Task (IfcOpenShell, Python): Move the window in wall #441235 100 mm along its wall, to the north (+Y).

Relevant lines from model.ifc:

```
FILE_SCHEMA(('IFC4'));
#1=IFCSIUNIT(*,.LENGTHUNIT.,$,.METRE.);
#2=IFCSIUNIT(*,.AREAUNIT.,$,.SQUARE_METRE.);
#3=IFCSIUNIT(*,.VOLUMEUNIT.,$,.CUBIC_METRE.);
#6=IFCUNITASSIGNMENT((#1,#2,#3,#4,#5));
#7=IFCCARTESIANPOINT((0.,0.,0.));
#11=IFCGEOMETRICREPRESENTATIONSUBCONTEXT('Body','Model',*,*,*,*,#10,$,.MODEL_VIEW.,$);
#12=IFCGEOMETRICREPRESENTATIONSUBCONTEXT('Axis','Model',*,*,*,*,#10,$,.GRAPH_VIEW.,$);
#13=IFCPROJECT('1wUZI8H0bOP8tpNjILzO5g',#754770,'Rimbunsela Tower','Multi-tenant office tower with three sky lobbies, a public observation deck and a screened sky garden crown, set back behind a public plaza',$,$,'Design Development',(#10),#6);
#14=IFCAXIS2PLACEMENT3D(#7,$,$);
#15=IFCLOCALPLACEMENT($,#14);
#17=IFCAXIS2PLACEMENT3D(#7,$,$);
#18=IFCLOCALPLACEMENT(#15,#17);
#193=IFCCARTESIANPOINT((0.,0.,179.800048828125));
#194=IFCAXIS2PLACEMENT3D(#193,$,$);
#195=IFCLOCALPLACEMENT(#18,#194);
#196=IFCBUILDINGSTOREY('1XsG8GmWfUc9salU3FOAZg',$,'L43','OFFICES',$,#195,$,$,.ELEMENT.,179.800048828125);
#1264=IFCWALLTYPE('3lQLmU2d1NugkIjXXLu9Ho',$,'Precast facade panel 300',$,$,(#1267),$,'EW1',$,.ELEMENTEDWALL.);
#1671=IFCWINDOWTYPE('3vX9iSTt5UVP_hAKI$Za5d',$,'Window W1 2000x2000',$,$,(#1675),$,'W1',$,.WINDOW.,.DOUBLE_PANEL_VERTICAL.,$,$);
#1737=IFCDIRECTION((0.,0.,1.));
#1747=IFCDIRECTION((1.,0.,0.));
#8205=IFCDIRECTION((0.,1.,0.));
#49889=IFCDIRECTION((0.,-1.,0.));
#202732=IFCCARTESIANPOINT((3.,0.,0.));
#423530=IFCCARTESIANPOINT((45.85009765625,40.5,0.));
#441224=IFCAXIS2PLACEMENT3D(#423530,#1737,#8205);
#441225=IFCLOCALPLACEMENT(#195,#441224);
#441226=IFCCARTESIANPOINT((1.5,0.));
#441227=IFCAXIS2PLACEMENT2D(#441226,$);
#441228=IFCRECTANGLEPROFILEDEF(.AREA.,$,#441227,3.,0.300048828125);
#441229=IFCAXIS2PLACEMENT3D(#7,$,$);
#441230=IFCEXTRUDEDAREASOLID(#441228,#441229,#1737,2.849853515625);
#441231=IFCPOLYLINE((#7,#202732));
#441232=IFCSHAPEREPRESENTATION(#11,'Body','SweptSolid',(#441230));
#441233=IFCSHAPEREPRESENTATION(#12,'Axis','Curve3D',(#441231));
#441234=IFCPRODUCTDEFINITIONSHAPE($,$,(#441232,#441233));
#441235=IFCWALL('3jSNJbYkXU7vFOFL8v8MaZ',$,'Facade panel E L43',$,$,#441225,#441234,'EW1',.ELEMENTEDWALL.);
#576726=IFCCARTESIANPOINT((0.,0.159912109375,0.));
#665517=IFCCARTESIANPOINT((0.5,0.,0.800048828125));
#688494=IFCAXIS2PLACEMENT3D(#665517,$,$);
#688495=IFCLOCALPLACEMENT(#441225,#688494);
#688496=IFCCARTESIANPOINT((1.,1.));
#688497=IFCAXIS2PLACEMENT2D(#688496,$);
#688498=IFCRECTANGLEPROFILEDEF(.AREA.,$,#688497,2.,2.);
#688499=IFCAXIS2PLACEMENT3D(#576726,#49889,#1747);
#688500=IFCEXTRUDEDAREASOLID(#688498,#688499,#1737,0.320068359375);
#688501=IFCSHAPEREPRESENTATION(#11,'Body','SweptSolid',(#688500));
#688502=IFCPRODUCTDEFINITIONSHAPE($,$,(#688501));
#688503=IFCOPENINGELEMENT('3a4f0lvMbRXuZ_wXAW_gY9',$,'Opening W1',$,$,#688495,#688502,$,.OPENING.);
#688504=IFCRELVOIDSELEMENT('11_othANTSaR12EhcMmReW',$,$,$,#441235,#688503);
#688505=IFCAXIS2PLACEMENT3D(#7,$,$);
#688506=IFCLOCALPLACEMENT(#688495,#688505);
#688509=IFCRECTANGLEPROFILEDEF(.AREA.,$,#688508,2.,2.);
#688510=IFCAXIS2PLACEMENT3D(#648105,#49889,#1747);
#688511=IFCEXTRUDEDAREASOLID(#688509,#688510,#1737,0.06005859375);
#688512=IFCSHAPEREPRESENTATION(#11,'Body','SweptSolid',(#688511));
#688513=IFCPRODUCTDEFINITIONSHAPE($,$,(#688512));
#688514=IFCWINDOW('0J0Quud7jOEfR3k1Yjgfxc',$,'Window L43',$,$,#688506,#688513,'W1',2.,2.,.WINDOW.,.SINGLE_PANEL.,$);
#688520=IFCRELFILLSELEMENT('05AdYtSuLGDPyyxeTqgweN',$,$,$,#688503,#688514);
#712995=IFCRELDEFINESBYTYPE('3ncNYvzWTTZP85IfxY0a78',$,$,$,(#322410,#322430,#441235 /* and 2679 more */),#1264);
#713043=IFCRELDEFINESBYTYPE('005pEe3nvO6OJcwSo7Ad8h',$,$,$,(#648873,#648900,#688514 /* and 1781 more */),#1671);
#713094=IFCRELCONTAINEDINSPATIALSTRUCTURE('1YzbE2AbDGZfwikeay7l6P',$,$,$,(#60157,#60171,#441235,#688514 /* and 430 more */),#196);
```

```python
import ifcopenshell
import ifcopenshell.api.geometry
import ifcopenshell.util.placement
import ifcopenshell.util.unit

model = ifcopenshell.open("model.ifc")
unit_scale = ifcopenshell.util.unit.calculate_unit_scale(model)

window = model.by_guid("0J0Quud7jOEfR3k1Yjgfxc")
opening = window.FillsVoids[0].RelatingOpeningElement
wall = opening.VoidsElements[0].RelatingBuildingElement

wall_matrix = ifcopenshell.util.placement.get_local_placement(wall.ObjectPlacement)
shift = wall_matrix[:3, 0] * 0.1 / unit_scale
before = ifcopenshell.util.placement.get_local_placement(window.ObjectPlacement)[:3, 3].copy()

# The window is placed relative to its opening, so it follows when the opening moves.
matrix = ifcopenshell.util.placement.get_local_placement(opening.ObjectPlacement)
matrix[:3, 3] += shift
ifcopenshell.api.geometry.edit_object_placement(
    model, product=opening, matrix=matrix, is_si=False, should_transform_children=True
)

after = ifcopenshell.util.placement.get_local_placement(window.ObjectPlacement)[:3, 3]
print("window moved by", (after - before).round(3) + 0.0)

model.write("model_v2.ifc")
```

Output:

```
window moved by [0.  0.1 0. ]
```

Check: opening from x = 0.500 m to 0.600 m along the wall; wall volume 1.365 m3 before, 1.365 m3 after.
